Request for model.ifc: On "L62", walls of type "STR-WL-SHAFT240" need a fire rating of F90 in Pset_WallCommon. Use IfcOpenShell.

First a look at what the model holds.

```python
import ifcopenshell
import ifcopenshell.util.element

model = ifcopenshell.open("model.ifc")
print(model.schema)
storey = next(s for s in model.by_type("IfcBuildingStorey") if s.Name == "L62")
walls = [e for e in ifcopenshell.util.element.get_decomposition(storey) if e.is_a("IfcWall")]
seen = {}
for e in walls:
    element_type = ifcopenshell.util.element.get_type(e)
    key = (element_type.Name if element_type != e and element_type else None, ifcopenshell.util.element.get_pset(e, "Pset_WallCommon", "FireRating"))
    seen[key] = seen.get(key, 0) + 1
for (name, value), count in sorted(seen.items(), key=str):
    print(count, "x", name, "|", value)
```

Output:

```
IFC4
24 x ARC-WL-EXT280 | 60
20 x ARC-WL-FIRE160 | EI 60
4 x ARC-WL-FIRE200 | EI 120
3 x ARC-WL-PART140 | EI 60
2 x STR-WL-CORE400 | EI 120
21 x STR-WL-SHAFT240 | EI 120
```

```python
import ifcopenshell
import ifcopenshell.api.pset
import ifcopenshell.util.element

model = ifcopenshell.open("model.ifc")

storey = next(s for s in model.by_type("IfcBuildingStorey") if s.Name == "L62")
walls = [e for e in ifcopenshell.util.element.get_decomposition(storey) if e.is_a("IfcWall")]

count = 0
for e in walls:
    element_type = ifcopenshell.util.element.get_type(e)
    if element_type in (None, e) or element_type.Name != "STR-WL-SHAFT240":
        continue
    found = ifcopenshell.util.element.get_pset(e, "Pset_WallCommon", should_inherit=False)
    if found:
        pset = model.by_id(found["id"])
        if len(ifcopenshell.util.element.get_elements_by_pset(pset)) > 1:
            pset = ifcopenshell.api.pset.unshare_pset(model, products=[e], pset=pset)[0]
    else:
        pset = ifcopenshell.api.pset.add_pset(model, product=e, name="Pset_WallCommon")
    ifcopenshell.api.pset.edit_pset(model, pset=pset, properties={"FireRating": "F90"})
    count += 1

print(count, "walls updated")

model.write("model-out.ifc")
```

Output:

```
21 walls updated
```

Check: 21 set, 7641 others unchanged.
